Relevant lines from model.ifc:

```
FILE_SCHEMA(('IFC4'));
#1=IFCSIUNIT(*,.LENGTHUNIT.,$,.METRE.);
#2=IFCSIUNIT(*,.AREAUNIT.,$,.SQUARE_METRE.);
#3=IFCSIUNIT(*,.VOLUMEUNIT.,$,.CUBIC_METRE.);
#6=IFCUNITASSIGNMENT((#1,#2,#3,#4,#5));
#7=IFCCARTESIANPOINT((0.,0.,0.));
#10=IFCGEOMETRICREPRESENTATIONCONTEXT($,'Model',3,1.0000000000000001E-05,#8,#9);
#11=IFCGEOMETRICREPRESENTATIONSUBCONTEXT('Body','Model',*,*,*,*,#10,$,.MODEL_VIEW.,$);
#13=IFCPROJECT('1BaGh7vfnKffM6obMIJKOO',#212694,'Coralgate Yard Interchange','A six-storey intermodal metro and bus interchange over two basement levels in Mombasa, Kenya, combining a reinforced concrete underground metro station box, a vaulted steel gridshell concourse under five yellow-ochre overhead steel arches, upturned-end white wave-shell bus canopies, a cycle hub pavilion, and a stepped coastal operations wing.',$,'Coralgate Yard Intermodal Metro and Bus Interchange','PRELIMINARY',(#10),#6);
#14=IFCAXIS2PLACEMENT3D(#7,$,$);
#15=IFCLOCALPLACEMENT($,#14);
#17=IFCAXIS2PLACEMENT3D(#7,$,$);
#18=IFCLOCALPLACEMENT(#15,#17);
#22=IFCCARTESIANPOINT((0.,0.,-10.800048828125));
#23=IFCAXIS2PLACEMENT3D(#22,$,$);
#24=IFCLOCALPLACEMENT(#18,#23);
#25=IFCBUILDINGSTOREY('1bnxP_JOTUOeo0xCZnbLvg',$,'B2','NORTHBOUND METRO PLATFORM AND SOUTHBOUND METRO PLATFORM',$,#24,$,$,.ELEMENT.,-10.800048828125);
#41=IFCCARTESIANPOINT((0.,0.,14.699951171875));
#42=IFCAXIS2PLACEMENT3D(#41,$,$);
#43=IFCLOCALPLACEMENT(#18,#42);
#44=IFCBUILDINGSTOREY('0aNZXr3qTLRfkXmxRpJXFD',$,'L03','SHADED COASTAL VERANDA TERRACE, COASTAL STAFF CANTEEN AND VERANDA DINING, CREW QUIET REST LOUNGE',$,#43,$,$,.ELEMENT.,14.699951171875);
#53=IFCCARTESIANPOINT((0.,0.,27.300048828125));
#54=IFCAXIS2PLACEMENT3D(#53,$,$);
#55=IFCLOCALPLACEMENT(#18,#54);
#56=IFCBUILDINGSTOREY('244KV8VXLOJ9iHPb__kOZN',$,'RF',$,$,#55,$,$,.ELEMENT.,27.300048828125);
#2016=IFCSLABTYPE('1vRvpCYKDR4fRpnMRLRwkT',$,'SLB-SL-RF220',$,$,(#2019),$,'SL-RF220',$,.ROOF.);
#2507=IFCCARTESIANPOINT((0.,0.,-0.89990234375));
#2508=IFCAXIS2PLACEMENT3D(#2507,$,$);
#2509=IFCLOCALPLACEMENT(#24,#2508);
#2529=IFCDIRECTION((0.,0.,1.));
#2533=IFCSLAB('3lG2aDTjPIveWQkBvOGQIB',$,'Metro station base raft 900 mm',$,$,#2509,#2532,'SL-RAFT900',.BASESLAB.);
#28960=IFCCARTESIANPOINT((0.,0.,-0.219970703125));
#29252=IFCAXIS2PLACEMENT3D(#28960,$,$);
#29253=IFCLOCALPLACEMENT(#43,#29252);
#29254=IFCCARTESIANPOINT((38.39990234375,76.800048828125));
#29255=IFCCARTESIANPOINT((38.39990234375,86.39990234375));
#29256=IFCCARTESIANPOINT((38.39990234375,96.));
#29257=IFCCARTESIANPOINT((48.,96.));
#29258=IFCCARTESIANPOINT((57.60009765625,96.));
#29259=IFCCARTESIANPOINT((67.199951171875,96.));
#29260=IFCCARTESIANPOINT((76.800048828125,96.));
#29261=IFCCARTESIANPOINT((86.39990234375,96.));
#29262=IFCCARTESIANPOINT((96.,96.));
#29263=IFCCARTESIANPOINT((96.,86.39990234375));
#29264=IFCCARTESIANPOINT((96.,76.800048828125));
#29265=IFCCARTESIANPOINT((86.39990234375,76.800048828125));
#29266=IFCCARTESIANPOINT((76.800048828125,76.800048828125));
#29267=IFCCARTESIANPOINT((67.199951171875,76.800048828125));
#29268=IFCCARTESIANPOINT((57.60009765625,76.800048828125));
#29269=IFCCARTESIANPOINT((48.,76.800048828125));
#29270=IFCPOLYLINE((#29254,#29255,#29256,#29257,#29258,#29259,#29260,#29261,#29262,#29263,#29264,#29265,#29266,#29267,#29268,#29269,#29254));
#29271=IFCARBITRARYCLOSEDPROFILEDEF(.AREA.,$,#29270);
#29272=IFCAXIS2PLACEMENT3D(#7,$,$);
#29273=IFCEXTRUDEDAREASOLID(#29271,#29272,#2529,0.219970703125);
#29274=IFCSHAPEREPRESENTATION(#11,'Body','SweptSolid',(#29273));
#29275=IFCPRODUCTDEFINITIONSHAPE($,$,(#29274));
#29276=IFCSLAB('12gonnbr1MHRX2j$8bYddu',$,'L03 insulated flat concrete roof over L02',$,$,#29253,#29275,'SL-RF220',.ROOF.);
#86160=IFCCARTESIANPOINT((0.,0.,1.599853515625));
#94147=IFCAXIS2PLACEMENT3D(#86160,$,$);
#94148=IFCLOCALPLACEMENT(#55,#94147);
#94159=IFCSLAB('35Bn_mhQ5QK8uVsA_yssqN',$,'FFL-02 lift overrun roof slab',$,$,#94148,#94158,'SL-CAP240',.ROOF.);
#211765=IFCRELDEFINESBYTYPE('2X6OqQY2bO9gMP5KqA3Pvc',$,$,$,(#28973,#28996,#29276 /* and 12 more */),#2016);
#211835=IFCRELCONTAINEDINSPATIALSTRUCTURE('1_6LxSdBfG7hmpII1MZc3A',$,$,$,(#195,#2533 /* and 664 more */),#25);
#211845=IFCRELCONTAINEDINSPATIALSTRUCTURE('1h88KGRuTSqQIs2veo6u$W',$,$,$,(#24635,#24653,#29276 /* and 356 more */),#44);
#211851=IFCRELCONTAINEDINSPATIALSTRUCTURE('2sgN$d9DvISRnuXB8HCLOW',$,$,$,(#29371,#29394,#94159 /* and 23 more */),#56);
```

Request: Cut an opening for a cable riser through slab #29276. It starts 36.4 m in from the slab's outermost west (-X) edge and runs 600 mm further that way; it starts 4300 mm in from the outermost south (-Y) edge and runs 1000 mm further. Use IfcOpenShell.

```python
import numpy as np
import ifcopenshell
import ifcopenshell.api.feature
import ifcopenshell.api.geometry
import ifcopenshell.api.root
import ifcopenshell.geom
import ifcopenshell.util.placement
import ifcopenshell.util.representation
import ifcopenshell.util.shape
import ifcopenshell.util.unit

model = ifcopenshell.open("model.ifc")
unit_scale = ifcopenshell.util.unit.calculate_unit_scale(model)
settings = ifcopenshell.geom.settings()


def volume(element):
    """Net volume in cubic metres, openings subtracted."""
    shape = ifcopenshell.geom.create_shape(settings, element)
    return ifcopenshell.util.shape.get_volume(shape.geometry)


slab = model.by_guid("12gonnbr1MHRX2j$8bYddu")
before = volume(slab)

# Extent in the slab's own axes, in metres. The edges named are its -X and -Y sides.
slab_shape = ifcopenshell.geom.create_shape(settings, slab)
vertices = ifcopenshell.util.shape.get_vertices(slab_shape.geometry)
x_min, y_min, bottom = vertices.min(axis=0)
top = vertices[:, 2].max()

opening = ifcopenshell.api.root.create_entity(model, ifc_class="IfcOpeningElement", name="Cable riser opening", predefined_type="OPENING")
context = ifcopenshell.util.representation.get_context(model, "Model", "Body", "MODEL_VIEW")
width, depth = 0.6, 1
outline = [(0.0, 0.0), (width, 0.0), (width, depth), (0.0, depth), (0.0, 0.0)]
# Overshoot both faces by 50 mm so the cut is clean.
shape = ifcopenshell.api.geometry.add_slab_representation(
    model, context=context, depth=top - bottom + 0.1, polyline=outline
)
ifcopenshell.api.geometry.assign_representation(model, product=opening, representation=shape)

matrix = ifcopenshell.util.placement.get_local_placement(slab.ObjectPlacement)
matrix[:, 3] = matrix @ np.append(np.array([x_min + 36.4, y_min + 4.3, bottom - 0.05]) / unit_scale, 1.0)
ifcopenshell.api.geometry.edit_object_placement(model, product=opening, matrix=matrix, is_si=False)
ifcopenshell.api.feature.add_feature(model, feature=opening, element=slab)

after = volume(slab)

print(f"slab volume {before:.3f} -> {after:.3f} m3")

model.write("model-out.ifc")
```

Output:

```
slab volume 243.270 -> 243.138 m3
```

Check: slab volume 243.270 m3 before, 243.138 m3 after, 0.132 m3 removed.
